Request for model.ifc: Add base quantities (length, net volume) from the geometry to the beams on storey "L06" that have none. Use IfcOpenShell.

First a look at what the model holds.

```python
import ifcopenshell
import ifcopenshell.util.element
import ifcopenshell.util.unit

model = ifcopenshell.open("model.ifc")
print(model.schema)
for unit_type in ("LENGTHUNIT", "AREAUNIT", "VOLUMEUNIT"):
    print(unit_type, ifcopenshell.util.unit.calculate_unit_scale(model, unit_type))
storey = next(s for s in model.by_type("IfcBuildingStorey") if s.Name == "L06")
beams = [e for e in ifcopenshell.util.element.get_decomposition(storey) if e.is_a("IfcBeam")]
for e in sorted(beams, key=lambda e: e.id()):
    print(e.id(), e.is_a(), e.Name, list(ifcopenshell.util.element.get_psets(e, qtos_only=True)), sep=" | ")
```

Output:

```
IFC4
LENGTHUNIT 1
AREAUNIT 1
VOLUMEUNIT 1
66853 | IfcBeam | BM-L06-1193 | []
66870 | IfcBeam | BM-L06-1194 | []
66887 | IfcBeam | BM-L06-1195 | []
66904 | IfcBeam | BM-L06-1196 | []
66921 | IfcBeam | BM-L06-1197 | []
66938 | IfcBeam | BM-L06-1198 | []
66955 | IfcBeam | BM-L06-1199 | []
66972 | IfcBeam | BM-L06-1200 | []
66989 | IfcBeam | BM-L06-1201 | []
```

```python
import ifcopenshell
import ifcopenshell.api.pset
import ifcopenshell.geom
import ifcopenshell.util.element
import ifcopenshell.util.shape
import ifcopenshell.util.unit

model = ifcopenshell.open("model.ifc")
unit_scale = ifcopenshell.util.unit.calculate_unit_scale(model)
volume_scale = ifcopenshell.util.unit.calculate_unit_scale(model, "VOLUMEUNIT")
settings = ifcopenshell.geom.settings()

storey = next(s for s in model.by_type("IfcBuildingStorey") if s.Name == "L06")
beams = [e for e in ifcopenshell.util.element.get_decomposition(storey) if e.is_a("IfcBeam")]

for e in sorted(beams, key=lambda e: e.id()):
    if ifcopenshell.util.element.get_psets(e, qtos_only=True, should_inherit=False):
        continue
    # Geometry comes back in metres, in the element's own axes.
    shape = ifcopenshell.geom.create_shape(settings, e)
    values = {
        "Length": ifcopenshell.util.shape.get_max_xyz(shape.geometry) / unit_scale,
        "NetVolume": ifcopenshell.util.shape.get_volume(shape.geometry) / volume_scale,
    }
    qto = ifcopenshell.api.pset.add_qto(model, product=e, name="Qto_BeamBaseQuantities")
    ifcopenshell.api.pset.edit_qto(model, qto=qto, properties=values)
    print(e.id(), {k: round(v, 3) for k, v in values.items()})

model.write("model-out.ifc")
```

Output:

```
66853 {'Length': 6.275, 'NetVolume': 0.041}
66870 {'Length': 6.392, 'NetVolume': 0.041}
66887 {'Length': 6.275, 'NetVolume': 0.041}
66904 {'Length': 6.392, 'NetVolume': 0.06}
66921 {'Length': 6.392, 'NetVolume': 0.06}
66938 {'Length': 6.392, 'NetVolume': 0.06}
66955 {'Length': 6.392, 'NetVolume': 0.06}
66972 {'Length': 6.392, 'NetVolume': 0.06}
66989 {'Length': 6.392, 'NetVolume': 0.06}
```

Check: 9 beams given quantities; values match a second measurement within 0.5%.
